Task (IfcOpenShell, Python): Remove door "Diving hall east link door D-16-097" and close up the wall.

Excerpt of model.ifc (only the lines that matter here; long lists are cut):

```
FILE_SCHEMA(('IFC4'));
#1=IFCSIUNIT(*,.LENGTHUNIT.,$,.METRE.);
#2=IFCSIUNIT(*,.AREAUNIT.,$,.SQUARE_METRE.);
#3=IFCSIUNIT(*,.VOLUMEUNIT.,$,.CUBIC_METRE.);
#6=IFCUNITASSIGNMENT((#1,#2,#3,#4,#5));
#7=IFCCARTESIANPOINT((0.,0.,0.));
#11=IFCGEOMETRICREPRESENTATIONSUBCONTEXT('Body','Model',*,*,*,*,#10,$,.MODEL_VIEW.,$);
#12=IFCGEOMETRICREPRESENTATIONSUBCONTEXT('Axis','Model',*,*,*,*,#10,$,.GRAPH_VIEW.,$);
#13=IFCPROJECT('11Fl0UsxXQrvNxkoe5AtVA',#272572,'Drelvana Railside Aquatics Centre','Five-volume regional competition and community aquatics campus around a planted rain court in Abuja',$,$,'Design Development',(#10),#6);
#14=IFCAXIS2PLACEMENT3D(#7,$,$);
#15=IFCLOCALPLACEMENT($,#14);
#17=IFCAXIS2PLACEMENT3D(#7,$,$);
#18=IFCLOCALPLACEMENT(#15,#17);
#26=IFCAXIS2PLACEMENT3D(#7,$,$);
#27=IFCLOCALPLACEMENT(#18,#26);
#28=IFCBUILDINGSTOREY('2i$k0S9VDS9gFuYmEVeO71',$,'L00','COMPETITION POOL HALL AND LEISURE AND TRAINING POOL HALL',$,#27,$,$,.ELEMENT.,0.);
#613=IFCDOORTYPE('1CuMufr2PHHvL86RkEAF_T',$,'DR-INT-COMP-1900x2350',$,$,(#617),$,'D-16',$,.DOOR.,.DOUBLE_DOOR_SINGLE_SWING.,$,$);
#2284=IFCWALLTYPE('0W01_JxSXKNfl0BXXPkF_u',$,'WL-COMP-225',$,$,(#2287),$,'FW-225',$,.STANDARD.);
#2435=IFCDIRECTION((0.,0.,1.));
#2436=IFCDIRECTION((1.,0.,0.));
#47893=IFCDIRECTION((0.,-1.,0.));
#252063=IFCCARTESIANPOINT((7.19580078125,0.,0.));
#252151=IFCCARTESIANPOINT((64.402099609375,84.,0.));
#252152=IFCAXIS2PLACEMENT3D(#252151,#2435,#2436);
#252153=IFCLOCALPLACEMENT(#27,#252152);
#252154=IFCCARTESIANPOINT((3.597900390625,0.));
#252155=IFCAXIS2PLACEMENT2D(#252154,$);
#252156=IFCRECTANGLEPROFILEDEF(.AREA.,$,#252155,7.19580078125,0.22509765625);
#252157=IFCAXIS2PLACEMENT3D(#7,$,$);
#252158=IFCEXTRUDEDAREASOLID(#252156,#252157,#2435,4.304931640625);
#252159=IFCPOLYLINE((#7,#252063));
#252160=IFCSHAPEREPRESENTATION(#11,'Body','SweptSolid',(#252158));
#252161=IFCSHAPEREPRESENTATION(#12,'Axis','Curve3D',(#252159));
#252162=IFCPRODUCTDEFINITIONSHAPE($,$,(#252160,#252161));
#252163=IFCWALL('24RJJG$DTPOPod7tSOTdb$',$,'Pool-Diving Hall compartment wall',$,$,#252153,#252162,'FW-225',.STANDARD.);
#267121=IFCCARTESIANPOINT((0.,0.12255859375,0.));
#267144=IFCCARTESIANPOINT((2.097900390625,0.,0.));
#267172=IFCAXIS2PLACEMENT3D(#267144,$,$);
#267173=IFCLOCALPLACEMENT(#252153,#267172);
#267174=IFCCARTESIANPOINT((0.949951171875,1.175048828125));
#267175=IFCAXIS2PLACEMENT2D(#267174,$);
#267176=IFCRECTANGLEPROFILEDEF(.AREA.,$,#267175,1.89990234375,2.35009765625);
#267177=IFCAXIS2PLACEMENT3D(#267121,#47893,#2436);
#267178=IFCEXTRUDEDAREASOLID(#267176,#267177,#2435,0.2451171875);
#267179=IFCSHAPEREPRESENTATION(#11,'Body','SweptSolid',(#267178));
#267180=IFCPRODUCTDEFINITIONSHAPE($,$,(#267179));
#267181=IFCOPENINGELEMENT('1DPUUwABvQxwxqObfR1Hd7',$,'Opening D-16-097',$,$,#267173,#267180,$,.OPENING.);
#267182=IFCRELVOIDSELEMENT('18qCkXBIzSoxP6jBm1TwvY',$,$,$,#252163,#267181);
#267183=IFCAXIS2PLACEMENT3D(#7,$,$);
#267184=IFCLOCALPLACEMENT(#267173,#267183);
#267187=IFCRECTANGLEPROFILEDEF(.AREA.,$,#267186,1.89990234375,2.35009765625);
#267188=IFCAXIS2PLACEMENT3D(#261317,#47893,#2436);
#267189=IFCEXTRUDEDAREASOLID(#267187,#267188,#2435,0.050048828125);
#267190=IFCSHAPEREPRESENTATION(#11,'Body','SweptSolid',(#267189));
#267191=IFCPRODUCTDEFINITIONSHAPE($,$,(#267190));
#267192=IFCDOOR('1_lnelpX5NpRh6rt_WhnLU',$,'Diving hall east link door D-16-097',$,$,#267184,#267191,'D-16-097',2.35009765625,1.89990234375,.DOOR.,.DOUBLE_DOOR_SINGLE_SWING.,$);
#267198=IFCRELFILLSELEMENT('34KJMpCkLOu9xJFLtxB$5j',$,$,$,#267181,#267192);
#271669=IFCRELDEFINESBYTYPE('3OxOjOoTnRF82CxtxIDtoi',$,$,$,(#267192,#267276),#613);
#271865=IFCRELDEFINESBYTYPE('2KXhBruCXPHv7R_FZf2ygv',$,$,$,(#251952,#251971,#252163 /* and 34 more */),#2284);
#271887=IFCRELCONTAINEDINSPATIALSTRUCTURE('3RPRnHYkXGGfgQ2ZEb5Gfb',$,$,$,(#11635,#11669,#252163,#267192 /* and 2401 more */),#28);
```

```python
import ifcopenshell
import ifcopenshell.api.feature
import ifcopenshell.api.root
import ifcopenshell.geom
import ifcopenshell.util.shape

model = ifcopenshell.open("model.ifc")
settings = ifcopenshell.geom.settings()


def volume(element):
    """Net volume in cubic metres, openings subtracted."""
    shape = ifcopenshell.geom.create_shape(settings, element)
    return ifcopenshell.util.shape.get_volume(shape.geometry)


door = model.by_id(267192)
opening = door.FillsVoids[0].RelatingOpeningElement
wall = opening.VoidsElements[0].RelatingBuildingElement
before = volume(wall)

ifcopenshell.api.root.remove_product(model, product=door)
ifcopenshell.api.feature.remove_feature(model, feature=opening)

after = volume(wall)

print(f"wall volume {before:.3f} -> {after:.3f} m3")

model.write("model_edited.ifc")
```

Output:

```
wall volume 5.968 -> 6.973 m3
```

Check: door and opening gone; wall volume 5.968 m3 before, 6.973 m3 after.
